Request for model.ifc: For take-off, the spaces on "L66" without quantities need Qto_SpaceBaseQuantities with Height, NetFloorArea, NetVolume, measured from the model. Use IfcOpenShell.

First a look at what the model holds.

```python
import ifcopenshell
import ifcopenshell.util.element
import ifcopenshell.util.unit

model = ifcopenshell.open("model.ifc")
print(model.schema)
for unit_type in ("LENGTHUNIT", "AREAUNIT", "VOLUMEUNIT"):
    print(unit_type, ifcopenshell.util.unit.calculate_unit_scale(model, unit_type))
storey = next(s for s in model.by_type("IfcBuildingStorey") if s.Name == "L66")
spaces = [e for e in ifcopenshell.util.element.get_decomposition(storey) if e.is_a("IfcSpace")]
for e in sorted(spaces, key=lambda e: e.id()):
    print(e.id(), e.is_a(), e.Name, list(ifcopenshell.util.element.get_psets(e, qtos_only=True)), sep=" | ")
```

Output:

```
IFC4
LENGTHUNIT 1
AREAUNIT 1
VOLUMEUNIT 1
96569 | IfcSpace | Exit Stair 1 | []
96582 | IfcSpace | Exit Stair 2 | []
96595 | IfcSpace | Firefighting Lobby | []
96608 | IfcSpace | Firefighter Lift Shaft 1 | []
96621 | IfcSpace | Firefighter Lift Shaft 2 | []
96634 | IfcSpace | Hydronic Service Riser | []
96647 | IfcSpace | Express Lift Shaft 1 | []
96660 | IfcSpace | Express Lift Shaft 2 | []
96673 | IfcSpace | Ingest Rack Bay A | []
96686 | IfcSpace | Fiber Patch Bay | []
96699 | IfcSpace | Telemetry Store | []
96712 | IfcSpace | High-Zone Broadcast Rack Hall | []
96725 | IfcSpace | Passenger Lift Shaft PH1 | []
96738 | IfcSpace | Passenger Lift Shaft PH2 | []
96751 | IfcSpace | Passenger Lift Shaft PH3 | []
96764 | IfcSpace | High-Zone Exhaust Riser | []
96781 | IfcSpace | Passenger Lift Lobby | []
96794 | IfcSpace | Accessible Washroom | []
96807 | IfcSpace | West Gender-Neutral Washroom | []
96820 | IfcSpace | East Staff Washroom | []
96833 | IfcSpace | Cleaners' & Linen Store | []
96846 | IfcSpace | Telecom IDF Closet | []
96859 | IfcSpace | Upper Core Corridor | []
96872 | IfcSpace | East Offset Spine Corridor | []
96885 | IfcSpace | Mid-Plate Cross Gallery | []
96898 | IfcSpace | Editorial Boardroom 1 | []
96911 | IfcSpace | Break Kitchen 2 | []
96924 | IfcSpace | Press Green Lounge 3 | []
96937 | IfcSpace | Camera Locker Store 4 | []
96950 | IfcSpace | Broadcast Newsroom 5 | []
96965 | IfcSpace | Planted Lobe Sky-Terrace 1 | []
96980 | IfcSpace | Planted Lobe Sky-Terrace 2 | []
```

```python
import ifcopenshell
import ifcopenshell.api.pset
import ifcopenshell.geom
import ifcopenshell.util.element
import ifcopenshell.util.shape
import ifcopenshell.util.unit

model = ifcopenshell.open("model.ifc")
unit_scale = ifcopenshell.util.unit.calculate_unit_scale(model)
area_scale = ifcopenshell.util.unit.calculate_unit_scale(model, "AREAUNIT")
volume_scale = ifcopenshell.util.unit.calculate_unit_scale(model, "VOLUMEUNIT")
settings = ifcopenshell.geom.settings()

storey = next(s for s in model.by_type("IfcBuildingStorey") if s.Name == "L66")
spaces = [e for e in ifcopenshell.util.element.get_decomposition(storey) if e.is_a("IfcSpace")]

for e in sorted(spaces, key=lambda e: e.id()):
    if ifcopenshell.util.element.get_psets(e, qtos_only=True, should_inherit=False):
        continue
    # Geometry comes back in metres, in the element's own axes.
    shape = ifcopenshell.geom.create_shape(settings, e)
    values = {
        "Height": ifcopenshell.util.shape.get_z(shape.geometry) / unit_scale,
        "NetFloorArea": ifcopenshell.util.shape.get_footprint_area(shape.geometry) / area_scale,
        "NetVolume": ifcopenshell.util.shape.get_volume(shape.geometry) / volume_scale,
    }
    qto = ifcopenshell.api.pset.add_qto(model, product=e, name="Qto_SpaceBaseQuantities")
    ifcopenshell.api.pset.edit_qto(model, qto=qto, properties=values)
    print(e.id(), {k: round(v, 3) for k, v in values.items()})

model.write("model-out.ifc")
```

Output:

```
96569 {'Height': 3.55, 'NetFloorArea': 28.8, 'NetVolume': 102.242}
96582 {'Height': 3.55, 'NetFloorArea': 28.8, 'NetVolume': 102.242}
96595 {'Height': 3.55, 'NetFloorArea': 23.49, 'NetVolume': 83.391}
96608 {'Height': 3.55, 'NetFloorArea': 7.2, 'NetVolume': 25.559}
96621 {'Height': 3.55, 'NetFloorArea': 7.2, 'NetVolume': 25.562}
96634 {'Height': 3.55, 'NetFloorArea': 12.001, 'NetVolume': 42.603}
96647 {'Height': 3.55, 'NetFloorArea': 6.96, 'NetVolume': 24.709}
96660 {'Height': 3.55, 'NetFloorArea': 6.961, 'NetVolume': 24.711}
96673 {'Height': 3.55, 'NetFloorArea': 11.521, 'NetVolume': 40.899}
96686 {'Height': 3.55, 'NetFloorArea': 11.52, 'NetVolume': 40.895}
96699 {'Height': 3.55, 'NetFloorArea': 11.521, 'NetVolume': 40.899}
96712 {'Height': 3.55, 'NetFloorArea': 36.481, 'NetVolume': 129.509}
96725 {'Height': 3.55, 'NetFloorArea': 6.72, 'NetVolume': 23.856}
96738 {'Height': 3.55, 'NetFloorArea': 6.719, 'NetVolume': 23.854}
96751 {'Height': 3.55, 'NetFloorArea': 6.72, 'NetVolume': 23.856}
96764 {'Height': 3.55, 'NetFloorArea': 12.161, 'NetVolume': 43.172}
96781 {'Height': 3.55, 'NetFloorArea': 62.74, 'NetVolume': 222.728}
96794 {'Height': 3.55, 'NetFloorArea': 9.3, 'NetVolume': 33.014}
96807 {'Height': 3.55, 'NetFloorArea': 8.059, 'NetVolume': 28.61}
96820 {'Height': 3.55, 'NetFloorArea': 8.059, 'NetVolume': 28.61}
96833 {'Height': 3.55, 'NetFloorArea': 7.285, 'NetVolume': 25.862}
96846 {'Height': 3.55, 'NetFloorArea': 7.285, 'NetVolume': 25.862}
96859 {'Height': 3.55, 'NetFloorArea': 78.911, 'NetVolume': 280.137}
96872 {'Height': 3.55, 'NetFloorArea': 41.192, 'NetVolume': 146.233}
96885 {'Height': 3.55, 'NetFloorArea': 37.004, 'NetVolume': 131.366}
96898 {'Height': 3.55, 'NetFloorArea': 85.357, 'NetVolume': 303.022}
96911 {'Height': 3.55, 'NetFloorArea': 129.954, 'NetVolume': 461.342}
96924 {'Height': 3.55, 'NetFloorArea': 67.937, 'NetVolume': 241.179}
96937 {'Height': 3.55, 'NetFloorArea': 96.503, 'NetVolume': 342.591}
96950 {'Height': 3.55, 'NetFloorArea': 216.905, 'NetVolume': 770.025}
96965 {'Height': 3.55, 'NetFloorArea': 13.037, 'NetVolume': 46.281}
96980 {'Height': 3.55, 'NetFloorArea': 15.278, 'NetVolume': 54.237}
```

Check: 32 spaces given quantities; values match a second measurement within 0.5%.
